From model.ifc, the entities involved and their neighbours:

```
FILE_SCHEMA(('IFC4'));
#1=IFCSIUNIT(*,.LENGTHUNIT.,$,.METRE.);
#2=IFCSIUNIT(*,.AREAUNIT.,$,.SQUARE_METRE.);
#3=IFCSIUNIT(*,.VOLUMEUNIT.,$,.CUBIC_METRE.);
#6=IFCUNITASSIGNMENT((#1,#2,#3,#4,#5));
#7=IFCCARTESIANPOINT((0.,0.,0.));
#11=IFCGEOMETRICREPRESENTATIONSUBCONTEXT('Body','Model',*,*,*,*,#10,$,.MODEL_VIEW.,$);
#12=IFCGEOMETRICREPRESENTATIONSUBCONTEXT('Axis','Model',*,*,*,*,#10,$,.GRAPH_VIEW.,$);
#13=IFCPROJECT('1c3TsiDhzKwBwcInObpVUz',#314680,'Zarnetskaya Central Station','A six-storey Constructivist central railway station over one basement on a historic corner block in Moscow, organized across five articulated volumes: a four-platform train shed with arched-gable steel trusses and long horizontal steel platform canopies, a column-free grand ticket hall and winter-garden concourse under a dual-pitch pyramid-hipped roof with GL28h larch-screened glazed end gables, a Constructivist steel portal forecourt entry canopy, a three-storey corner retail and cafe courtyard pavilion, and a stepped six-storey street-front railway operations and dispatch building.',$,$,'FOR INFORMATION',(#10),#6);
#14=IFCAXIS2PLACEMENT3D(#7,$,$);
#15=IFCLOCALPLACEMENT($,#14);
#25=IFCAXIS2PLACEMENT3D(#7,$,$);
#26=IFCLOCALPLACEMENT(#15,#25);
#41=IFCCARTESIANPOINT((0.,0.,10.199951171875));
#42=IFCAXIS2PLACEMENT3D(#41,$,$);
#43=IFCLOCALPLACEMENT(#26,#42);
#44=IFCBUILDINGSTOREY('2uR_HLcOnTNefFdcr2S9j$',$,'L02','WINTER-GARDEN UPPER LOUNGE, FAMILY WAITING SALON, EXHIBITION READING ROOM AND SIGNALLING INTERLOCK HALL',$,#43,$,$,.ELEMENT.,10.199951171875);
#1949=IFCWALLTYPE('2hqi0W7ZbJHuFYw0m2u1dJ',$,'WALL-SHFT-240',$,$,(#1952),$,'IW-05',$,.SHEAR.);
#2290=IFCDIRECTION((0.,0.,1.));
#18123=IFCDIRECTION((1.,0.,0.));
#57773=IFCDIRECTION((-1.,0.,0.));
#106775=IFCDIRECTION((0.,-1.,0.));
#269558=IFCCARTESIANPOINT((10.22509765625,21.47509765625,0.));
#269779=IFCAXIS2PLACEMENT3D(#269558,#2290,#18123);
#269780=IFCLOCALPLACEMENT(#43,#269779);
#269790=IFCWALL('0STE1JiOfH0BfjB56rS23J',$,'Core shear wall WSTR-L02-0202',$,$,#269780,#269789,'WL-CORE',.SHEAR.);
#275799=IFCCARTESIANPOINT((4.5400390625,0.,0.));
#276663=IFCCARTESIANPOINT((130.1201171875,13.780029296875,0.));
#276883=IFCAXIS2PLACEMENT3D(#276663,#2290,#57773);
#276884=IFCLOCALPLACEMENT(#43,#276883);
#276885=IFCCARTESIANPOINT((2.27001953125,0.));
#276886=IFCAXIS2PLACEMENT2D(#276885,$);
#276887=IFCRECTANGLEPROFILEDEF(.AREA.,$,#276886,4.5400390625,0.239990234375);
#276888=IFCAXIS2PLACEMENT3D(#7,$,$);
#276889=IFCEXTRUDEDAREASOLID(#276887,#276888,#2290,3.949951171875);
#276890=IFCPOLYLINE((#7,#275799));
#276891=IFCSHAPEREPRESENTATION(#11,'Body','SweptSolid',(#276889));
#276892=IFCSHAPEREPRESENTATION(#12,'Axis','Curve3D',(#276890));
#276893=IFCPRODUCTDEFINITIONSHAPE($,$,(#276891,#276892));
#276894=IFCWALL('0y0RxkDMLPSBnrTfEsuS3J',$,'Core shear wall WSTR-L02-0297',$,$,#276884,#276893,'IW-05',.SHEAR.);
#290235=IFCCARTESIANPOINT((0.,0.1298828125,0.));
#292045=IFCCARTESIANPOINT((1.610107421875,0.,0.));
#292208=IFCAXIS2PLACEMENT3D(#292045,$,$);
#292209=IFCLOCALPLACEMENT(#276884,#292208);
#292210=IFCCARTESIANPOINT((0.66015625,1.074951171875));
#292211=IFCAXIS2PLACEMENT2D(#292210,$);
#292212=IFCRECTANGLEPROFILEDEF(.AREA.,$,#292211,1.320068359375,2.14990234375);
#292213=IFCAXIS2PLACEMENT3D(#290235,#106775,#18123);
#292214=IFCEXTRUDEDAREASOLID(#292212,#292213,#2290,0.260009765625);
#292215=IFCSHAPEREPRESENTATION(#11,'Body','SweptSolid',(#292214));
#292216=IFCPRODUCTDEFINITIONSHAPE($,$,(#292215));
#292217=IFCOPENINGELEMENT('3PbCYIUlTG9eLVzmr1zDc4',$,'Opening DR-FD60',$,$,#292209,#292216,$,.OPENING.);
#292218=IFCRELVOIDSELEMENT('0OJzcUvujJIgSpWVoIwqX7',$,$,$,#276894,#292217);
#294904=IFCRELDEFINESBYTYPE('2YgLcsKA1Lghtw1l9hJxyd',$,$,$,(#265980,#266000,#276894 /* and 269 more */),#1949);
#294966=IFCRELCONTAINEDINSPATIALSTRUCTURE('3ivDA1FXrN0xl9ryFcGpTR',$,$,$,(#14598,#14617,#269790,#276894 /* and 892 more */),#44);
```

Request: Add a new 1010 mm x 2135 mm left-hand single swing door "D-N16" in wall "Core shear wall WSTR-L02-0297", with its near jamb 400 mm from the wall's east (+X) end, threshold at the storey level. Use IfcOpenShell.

```python
import numpy as np
import ifcopenshell
import ifcopenshell.api.feature
import ifcopenshell.api.geometry
import ifcopenshell.api.root
import ifcopenshell.api.spatial
import ifcopenshell.geom
import ifcopenshell.util.element
import ifcopenshell.util.placement
import ifcopenshell.util.representation
import ifcopenshell.util.shape
import ifcopenshell.util.unit

model = ifcopenshell.open("model.ifc")
unit_scale = ifcopenshell.util.unit.calculate_unit_scale(model)
settings = ifcopenshell.geom.settings()


def volume(element):
    """Net volume in cubic metres, openings subtracted."""
    shape = ifcopenshell.geom.create_shape(settings, element)
    return ifcopenshell.util.shape.get_volume(shape.geometry)


wall = model.by_id(276894)
storey = ifcopenshell.util.element.get_container(wall, ifc_class="IfcBuildingStorey")
context = ifcopenshell.util.representation.get_context(model, "Model", "Body", "MODEL_VIEW")
before = volume(wall)

width, height, from_end, sill = 1.01, 2.135, 0.4, 0.0  # metres

# The wall runs along its own X axis, and the end named is its -X end.
wall_shape = ifcopenshell.geom.create_shape(settings, wall)
x, y, z = ifcopenshell.util.shape.get_vertices(wall_shape.geometry).T
start = x.min() + from_end
face, thickness = float(y.min()), float(y.max() - y.min())
wall_matrix = ifcopenshell.util.placement.get_local_placement(wall.ObjectPlacement)
level = ifcopenshell.util.placement.get_local_placement(storey.ObjectPlacement)[2, 3]


def in_wall(x, y):
    """Placement at x, y metres in the wall's axes, at sill height."""
    matrix = wall_matrix.copy()
    matrix[:, 3] = wall_matrix @ np.array([x / unit_scale, y / unit_scale, 0.0, 1.0])
    matrix[2, 3] = level + sill / unit_scale
    return matrix


# Opening: a box that overshoots both wall faces by 50 mm.
opening = ifcopenshell.api.root.create_entity(model, ifc_class="IfcOpeningElement", predefined_type="OPENING")
box = ifcopenshell.api.geometry.add_wall_representation(
    model, context=context, length=width, height=height, thickness=thickness + 0.1
)
ifcopenshell.api.geometry.assign_representation(model, product=opening, representation=box)
ifcopenshell.api.geometry.edit_object_placement(model, product=opening, matrix=in_wall(start, face - 0.05), is_si=False)
ifcopenshell.api.feature.add_feature(model, feature=opening, element=wall)

door = ifcopenshell.api.root.create_entity(model, ifc_class="IfcDoor", name="D-N16", predefined_type="DOOR")
door.OverallWidth, door.OverallHeight = width / unit_scale, height / unit_scale
door.OperationType = "SINGLE_SWING_LEFT"
body = ifcopenshell.api.geometry.add_door_representation(
    model,
    context=context,
    overall_width=door.OverallWidth,
    overall_height=door.OverallHeight,
    operation_type="SINGLE_SWING_LEFT",
    lining_properties={"LiningDepth": thickness / unit_scale, "ThresholdDepth": thickness / unit_scale},
)
ifcopenshell.api.geometry.assign_representation(model, product=door, representation=body)
ifcopenshell.api.spatial.assign_container(model, products=[door], relating_structure=storey)
ifcopenshell.api.feature.add_filling(model, opening=opening, element=door)

# The lining spans the wall, so the door starts at the wall face.
ifcopenshell.api.geometry.edit_object_placement(model, product=door, matrix=in_wall(start, face), is_si=False)

after = volume(wall)

print(f"wall volume {before:.3f} -> {after:.3f} m3")

model.write("model-out.ifc")
```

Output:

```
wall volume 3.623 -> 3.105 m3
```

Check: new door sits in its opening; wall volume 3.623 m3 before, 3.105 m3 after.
